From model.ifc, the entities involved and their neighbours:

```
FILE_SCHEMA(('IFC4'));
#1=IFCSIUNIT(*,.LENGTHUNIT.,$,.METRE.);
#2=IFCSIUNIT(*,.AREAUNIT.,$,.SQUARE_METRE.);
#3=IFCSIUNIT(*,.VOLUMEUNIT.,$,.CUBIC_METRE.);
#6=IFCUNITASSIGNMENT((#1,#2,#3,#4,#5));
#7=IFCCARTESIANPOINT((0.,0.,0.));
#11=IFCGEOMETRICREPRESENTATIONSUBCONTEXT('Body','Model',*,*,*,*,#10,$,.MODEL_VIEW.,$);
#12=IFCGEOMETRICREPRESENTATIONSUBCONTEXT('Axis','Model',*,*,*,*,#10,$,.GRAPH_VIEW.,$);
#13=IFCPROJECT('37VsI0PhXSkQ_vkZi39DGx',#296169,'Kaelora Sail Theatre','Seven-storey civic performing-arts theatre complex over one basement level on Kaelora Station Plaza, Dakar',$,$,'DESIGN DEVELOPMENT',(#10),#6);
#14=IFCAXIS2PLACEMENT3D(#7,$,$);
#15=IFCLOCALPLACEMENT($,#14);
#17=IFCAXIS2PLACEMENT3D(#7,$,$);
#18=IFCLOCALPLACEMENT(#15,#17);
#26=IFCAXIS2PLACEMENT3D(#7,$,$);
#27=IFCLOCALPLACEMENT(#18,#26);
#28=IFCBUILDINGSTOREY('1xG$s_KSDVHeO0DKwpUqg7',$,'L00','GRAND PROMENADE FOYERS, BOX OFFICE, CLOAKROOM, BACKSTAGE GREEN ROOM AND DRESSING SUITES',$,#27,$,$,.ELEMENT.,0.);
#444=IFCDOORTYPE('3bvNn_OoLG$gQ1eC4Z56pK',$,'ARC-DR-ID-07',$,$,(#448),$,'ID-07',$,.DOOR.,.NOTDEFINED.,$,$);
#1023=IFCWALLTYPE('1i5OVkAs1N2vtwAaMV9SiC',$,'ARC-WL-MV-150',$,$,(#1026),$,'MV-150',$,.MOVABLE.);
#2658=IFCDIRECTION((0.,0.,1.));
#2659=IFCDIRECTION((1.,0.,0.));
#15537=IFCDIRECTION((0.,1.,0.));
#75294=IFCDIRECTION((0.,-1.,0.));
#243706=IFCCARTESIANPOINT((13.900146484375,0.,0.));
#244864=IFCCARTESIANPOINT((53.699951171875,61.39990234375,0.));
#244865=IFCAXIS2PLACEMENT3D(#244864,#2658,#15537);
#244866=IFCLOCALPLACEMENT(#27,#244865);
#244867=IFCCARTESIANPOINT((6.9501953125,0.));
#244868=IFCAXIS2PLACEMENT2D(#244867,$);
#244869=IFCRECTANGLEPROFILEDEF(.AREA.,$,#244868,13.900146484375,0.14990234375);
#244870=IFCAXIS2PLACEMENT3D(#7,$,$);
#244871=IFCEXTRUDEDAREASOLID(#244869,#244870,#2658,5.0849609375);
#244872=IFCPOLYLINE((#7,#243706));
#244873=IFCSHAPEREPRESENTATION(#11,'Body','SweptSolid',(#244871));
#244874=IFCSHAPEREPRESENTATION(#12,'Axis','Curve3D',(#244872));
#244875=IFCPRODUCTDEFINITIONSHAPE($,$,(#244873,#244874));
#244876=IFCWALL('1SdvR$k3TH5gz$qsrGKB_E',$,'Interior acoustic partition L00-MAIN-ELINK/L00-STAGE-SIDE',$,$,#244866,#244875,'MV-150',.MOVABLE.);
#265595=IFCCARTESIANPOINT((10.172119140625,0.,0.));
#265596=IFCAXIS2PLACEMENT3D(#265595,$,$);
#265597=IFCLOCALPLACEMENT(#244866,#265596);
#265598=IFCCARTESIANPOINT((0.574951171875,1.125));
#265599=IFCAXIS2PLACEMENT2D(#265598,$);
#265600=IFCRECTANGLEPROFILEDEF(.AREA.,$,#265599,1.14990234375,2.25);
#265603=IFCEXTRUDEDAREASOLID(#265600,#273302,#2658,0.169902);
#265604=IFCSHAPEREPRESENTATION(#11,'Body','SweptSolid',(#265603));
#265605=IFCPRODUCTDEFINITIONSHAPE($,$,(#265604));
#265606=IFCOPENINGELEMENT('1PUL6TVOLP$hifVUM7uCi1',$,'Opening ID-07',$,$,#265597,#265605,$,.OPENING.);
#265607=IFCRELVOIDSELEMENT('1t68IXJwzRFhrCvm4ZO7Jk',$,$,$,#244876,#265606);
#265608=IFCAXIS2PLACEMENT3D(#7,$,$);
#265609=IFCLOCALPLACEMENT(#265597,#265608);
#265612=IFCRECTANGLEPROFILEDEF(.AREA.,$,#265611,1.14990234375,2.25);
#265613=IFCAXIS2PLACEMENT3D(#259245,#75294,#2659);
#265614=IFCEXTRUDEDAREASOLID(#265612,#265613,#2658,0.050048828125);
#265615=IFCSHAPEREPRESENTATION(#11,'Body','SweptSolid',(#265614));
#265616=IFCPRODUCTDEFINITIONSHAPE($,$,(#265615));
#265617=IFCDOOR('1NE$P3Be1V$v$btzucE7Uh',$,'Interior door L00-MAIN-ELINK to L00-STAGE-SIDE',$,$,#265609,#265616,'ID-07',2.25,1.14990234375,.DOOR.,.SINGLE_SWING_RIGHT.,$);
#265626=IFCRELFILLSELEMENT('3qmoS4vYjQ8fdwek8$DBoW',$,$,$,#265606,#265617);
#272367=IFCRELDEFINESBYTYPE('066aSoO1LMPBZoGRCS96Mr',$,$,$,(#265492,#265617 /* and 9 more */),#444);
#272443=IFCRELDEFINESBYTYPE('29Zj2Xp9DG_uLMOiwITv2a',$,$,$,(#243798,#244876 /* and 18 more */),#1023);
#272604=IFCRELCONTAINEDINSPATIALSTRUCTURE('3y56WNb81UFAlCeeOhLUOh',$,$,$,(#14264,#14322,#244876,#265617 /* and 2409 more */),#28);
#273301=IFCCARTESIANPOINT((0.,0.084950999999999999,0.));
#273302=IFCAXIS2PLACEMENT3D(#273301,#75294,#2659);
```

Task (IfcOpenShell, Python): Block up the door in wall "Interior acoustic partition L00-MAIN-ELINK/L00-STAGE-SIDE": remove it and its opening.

```python
import ifcopenshell
import ifcopenshell.api.feature
import ifcopenshell.api.root
import ifcopenshell.geom
import ifcopenshell.util.shape

model = ifcopenshell.open("model.ifc")
settings = ifcopenshell.geom.settings()


def volume(element):
    """Net volume in cubic metres, openings subtracted."""
    shape = ifcopenshell.geom.create_shape(settings, element)
    return ifcopenshell.util.shape.get_volume(shape.geometry)


door = model.by_guid("1NE$P3Be1V$v$btzucE7Uh")
opening = door.FillsVoids[0].RelatingOpeningElement
wall = opening.VoidsElements[0].RelatingBuildingElement
before = volume(wall)

ifcopenshell.api.root.remove_product(model, product=door)
ifcopenshell.api.feature.remove_feature(model, feature=opening)

after = volume(wall)

print(f"wall volume {before:.3f} -> {after:.3f} m3")

model.write("model_edited.ifc")
```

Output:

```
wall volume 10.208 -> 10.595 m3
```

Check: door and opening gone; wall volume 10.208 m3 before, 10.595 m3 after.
